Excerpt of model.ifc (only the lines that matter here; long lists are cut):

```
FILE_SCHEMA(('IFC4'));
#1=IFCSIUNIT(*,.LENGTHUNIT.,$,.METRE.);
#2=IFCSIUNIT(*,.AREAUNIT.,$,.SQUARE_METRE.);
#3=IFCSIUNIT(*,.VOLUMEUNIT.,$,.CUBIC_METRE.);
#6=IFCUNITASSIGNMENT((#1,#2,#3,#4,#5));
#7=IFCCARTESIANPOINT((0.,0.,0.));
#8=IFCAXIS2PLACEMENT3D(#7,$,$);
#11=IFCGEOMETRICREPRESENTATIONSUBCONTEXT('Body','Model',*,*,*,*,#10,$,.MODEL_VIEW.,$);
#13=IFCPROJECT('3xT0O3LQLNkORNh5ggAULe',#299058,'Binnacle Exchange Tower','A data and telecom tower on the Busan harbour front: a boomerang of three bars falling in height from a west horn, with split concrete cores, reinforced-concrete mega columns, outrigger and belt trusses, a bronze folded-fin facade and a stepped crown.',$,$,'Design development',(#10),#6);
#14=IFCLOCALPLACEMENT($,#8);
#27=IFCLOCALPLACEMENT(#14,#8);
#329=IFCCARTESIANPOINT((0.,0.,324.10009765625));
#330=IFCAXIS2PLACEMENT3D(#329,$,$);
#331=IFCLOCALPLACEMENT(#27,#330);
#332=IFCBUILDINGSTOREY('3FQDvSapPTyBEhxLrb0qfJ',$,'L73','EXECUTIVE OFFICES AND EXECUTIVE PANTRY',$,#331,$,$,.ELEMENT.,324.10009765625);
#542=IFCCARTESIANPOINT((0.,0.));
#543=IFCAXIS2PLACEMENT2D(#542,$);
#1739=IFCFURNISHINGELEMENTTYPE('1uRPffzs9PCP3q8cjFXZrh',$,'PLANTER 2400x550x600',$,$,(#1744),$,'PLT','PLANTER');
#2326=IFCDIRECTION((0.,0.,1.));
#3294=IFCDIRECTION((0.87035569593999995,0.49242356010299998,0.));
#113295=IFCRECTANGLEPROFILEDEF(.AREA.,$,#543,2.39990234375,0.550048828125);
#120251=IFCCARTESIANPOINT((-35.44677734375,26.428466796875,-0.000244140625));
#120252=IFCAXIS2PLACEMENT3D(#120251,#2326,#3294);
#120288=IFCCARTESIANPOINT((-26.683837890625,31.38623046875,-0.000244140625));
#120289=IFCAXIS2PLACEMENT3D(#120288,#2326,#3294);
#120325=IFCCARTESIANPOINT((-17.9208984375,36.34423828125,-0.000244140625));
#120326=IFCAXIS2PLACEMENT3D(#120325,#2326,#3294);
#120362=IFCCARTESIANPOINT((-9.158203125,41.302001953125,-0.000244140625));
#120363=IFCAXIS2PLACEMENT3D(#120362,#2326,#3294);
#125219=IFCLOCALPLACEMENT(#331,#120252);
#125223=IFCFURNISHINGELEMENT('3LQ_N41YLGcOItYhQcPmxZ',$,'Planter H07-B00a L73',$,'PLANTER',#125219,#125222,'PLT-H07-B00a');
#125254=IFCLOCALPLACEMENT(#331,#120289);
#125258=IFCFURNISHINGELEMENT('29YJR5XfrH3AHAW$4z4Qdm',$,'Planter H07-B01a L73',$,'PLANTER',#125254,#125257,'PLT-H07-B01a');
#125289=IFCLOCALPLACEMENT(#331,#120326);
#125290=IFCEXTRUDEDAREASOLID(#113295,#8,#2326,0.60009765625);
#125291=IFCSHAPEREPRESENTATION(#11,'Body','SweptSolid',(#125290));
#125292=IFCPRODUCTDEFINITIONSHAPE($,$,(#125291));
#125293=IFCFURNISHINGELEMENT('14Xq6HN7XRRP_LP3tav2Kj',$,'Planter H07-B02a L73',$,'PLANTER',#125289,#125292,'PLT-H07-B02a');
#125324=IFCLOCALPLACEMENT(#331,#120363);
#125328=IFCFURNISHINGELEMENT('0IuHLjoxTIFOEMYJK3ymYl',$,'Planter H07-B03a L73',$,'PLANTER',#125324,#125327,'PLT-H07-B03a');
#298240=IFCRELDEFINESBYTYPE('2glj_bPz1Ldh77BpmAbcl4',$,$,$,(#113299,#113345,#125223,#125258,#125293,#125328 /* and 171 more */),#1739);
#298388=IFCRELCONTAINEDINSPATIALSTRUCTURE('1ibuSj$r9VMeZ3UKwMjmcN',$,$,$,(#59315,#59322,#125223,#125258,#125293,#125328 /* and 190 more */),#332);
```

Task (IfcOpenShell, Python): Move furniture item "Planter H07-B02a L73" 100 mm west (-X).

```python
import ifcopenshell
import ifcopenshell.api.geometry
import ifcopenshell.util.placement

model = ifcopenshell.open("model.ifc")

item = model.by_guid("14Xq6HN7XRRP_LP3tav2Kj")
matrix = ifcopenshell.util.placement.get_local_placement(item.ObjectPlacement)
matrix[0, 3] -= 0.1
ifcopenshell.api.geometry.edit_object_placement(model, product=item, matrix=matrix, is_si=False)

print(ifcopenshell.util.placement.get_local_placement(item.ObjectPlacement).round(3) + 0.0)

model.write("model_updated.ifc")
```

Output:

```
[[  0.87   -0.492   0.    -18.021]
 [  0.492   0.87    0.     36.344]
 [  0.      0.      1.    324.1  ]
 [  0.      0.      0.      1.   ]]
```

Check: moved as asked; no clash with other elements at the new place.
